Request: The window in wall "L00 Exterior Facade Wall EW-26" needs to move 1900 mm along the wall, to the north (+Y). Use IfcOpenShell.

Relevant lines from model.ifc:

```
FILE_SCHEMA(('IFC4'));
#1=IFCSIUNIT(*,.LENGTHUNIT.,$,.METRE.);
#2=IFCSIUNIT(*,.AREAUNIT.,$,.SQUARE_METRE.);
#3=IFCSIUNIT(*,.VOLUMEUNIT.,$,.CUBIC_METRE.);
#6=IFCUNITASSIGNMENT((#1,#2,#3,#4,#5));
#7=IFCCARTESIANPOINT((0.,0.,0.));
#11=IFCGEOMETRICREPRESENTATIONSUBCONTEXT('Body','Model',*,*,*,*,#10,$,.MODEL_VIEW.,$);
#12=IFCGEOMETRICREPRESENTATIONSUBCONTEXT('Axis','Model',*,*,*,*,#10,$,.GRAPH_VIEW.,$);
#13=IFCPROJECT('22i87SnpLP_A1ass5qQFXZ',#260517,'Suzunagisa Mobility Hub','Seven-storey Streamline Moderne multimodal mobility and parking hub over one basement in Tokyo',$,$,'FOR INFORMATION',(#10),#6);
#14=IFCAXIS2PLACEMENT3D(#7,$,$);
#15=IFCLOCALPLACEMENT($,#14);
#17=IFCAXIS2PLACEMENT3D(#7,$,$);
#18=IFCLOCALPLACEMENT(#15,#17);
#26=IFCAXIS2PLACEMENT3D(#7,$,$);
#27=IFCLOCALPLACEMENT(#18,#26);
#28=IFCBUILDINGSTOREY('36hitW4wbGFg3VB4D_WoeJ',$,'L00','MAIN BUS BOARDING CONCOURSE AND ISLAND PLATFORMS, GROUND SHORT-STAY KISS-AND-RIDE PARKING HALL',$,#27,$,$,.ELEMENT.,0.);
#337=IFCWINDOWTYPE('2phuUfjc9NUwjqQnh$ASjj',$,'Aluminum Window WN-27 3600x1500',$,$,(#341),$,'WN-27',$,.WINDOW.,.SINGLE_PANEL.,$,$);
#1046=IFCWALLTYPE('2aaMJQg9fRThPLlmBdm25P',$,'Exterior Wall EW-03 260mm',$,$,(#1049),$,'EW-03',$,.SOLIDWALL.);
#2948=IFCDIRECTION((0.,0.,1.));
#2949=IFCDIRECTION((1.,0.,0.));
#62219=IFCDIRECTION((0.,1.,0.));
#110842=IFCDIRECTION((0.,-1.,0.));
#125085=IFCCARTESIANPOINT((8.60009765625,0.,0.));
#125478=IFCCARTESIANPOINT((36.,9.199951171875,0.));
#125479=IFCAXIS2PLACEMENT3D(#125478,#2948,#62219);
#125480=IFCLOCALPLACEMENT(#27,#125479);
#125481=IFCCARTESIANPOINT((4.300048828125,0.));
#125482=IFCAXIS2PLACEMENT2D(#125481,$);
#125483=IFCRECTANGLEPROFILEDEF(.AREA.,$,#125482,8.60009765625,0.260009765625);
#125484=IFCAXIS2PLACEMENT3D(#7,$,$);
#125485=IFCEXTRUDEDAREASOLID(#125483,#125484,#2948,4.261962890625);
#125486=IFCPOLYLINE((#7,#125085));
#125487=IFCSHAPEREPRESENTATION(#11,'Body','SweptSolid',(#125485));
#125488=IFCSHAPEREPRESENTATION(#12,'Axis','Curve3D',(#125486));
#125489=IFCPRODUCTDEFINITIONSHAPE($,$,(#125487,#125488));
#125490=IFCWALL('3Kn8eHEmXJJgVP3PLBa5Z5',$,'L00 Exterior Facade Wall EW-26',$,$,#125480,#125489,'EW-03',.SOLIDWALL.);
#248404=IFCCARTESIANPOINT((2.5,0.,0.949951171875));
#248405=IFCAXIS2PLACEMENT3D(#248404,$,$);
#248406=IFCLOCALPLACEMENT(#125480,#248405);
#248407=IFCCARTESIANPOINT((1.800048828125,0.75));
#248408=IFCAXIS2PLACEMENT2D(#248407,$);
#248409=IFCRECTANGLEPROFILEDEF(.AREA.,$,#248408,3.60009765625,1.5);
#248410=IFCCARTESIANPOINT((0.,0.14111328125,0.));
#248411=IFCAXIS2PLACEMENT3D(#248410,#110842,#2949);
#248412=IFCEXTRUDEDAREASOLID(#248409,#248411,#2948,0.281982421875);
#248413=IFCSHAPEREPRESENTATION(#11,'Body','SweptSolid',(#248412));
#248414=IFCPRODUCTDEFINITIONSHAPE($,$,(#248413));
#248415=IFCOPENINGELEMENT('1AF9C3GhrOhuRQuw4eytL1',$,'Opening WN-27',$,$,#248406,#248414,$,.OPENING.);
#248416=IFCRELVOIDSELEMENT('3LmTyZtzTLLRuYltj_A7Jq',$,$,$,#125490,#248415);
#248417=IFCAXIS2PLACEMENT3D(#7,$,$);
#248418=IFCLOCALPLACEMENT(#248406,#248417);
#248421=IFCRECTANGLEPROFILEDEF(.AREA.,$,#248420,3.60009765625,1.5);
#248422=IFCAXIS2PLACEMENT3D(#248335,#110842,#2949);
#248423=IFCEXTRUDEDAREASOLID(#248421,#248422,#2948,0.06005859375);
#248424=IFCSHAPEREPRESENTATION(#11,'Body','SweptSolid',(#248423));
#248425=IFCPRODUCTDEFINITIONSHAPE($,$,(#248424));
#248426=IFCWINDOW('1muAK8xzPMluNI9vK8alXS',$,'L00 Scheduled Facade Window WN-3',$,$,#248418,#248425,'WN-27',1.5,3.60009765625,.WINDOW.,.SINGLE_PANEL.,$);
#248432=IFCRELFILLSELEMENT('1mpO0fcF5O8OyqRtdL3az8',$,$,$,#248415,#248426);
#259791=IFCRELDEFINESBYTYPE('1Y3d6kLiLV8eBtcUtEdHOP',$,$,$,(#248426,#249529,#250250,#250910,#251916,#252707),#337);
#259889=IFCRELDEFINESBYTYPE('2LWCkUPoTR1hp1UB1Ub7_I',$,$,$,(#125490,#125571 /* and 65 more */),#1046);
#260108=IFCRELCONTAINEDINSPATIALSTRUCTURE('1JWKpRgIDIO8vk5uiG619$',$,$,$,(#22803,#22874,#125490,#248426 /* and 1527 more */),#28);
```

```python
import ifcopenshell
import ifcopenshell.api.geometry
import ifcopenshell.util.placement
import ifcopenshell.util.unit

model = ifcopenshell.open("model.ifc")
unit_scale = ifcopenshell.util.unit.calculate_unit_scale(model)

window = model.by_guid("1muAK8xzPMluNI9vK8alXS")
opening = window.FillsVoids[0].RelatingOpeningElement
wall = opening.VoidsElements[0].RelatingBuildingElement

wall_matrix = ifcopenshell.util.placement.get_local_placement(wall.ObjectPlacement)
shift = wall_matrix[:3, 0] * 1.9 / unit_scale
before = ifcopenshell.util.placement.get_local_placement(window.ObjectPlacement)[:3, 3].copy()

# The window is placed relative to its opening, so it follows when the opening moves.
matrix = ifcopenshell.util.placement.get_local_placement(opening.ObjectPlacement)
matrix[:3, 3] += shift
ifcopenshell.api.geometry.edit_object_placement(
    model, product=opening, matrix=matrix, is_si=False, should_transform_children=True
)

after = ifcopenshell.util.placement.get_local_placement(window.ObjectPlacement)[:3, 3]
print("window moved by", (after - before).round(3) + 0.0)

model.write("model_v2.ifc")
```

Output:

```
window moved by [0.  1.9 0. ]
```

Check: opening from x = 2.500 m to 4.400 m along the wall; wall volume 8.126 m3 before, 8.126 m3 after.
